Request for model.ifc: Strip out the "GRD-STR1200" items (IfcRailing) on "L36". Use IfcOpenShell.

First a look at what the model holds.

```python
import ifcopenshell
import ifcopenshell.util.element

model = ifcopenshell.open("model.ifc")
print(model.schema)
storey = next(s for s in model.by_type("IfcBuildingStorey") if s.Name == "L36")
railings = [e for e in ifcopenshell.util.element.get_decomposition(storey) if e.is_a("IfcRailing")]
seen = {}
for e in railings:
    element_type = ifcopenshell.util.element.get_type(e)
    name = element_type.Name if element_type not in (None, e) else None
    seen[name] = seen.get(name, 0) + 1
for name, count in sorted(seen.items(), key=str):
    print(count, "x", name)
```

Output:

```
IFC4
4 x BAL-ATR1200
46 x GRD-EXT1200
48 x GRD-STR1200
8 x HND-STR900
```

```python
import ifcopenshell
import ifcopenshell.api.root
import ifcopenshell.util.element

model = ifcopenshell.open("model.ifc")

storey = next(s for s in model.by_type("IfcBuildingStorey") if s.Name == "L36")
railings = [e for e in ifcopenshell.util.element.get_decomposition(storey) if e.is_a("IfcRailing")]
targets = [e for e in railings if (t := ifcopenshell.util.element.get_type(e)) not in (None, e) and t.Name == "GRD-STR1200"]

for e in targets:
    ifcopenshell.api.root.remove_product(model, product=e)
print(len(targets), "removed")

model.write("model-out.ifc")
```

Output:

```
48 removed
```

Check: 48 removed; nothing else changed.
